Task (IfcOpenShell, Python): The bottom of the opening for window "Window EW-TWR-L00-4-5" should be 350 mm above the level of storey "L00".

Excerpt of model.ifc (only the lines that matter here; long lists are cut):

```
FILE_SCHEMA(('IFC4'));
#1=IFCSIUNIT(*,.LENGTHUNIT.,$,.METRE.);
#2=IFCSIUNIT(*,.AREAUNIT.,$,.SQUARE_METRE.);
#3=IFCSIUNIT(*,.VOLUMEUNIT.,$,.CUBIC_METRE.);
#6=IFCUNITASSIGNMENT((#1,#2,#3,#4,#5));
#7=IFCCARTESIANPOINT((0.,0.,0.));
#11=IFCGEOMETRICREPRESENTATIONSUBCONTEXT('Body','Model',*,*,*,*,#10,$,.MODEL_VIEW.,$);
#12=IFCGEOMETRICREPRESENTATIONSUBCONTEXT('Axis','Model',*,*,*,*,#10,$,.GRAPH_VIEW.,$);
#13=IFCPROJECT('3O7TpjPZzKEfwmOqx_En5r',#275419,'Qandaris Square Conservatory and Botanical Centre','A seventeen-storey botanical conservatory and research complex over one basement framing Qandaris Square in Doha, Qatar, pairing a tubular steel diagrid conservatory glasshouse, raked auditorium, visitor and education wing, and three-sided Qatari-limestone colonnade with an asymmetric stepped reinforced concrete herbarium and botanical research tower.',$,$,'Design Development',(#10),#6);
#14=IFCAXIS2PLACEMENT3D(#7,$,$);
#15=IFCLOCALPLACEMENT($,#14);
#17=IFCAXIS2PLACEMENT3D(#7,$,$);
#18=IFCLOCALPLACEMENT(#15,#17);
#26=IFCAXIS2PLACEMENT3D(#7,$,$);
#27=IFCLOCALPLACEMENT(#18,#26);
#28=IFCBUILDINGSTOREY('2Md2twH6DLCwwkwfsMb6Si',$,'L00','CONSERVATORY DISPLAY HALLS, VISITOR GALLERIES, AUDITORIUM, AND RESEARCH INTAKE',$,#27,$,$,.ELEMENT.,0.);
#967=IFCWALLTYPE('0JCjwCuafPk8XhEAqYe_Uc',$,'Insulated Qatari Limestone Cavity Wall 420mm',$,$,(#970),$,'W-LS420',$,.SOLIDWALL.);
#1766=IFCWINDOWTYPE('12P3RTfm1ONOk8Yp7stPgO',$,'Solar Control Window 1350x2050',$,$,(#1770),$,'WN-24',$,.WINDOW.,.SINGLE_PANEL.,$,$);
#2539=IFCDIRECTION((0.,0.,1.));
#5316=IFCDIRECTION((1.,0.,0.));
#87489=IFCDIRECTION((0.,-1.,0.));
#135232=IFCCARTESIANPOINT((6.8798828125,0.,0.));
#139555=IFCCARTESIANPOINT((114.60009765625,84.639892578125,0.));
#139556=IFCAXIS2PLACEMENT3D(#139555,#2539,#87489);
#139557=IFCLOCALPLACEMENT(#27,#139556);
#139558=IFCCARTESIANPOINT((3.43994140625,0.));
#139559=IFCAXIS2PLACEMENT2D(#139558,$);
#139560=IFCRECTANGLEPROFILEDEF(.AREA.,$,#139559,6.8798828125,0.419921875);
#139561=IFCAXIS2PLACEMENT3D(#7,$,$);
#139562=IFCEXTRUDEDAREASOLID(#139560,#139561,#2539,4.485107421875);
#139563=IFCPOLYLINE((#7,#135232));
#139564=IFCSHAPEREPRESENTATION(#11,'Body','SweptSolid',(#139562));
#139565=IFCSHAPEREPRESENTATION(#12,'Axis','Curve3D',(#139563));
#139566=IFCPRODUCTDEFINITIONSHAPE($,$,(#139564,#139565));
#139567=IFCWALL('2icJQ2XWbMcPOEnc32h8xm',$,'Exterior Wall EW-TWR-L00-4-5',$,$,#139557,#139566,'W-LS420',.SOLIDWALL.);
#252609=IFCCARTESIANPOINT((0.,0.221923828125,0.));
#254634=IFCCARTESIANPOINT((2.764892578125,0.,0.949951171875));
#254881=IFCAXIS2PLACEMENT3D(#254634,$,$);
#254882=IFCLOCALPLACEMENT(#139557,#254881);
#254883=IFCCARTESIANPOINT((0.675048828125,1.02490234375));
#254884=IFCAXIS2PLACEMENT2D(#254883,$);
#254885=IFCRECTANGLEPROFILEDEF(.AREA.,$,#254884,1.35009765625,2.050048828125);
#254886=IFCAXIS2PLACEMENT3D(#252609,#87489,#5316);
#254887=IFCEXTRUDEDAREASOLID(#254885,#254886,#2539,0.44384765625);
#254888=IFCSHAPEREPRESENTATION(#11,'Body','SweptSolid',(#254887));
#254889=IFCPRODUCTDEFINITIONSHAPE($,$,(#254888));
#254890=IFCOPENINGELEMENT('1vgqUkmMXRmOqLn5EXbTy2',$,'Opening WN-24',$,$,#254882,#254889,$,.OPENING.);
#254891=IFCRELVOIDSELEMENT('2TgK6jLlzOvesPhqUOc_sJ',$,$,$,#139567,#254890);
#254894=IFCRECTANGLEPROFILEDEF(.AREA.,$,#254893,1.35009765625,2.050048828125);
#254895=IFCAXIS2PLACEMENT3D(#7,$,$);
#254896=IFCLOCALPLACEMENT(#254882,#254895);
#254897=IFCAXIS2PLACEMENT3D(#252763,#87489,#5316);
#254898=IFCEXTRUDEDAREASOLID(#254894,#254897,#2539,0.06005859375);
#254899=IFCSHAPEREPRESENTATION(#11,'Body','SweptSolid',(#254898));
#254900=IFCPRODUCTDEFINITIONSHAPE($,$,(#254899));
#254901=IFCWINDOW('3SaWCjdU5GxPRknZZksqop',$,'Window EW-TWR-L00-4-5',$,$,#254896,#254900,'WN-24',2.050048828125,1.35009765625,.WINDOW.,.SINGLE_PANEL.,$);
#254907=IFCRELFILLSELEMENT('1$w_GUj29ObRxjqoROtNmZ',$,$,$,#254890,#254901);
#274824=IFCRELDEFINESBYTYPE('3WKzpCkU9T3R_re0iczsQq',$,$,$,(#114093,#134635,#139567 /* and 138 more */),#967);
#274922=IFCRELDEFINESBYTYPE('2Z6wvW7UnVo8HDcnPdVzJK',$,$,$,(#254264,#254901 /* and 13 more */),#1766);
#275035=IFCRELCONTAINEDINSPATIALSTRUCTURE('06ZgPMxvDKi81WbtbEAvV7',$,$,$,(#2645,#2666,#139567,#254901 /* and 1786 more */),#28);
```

```python
import numpy as np
import ifcopenshell
import ifcopenshell.api.geometry
import ifcopenshell.geom
import ifcopenshell.util.element
import ifcopenshell.util.placement
import ifcopenshell.util.shape
import ifcopenshell.util.unit

model = ifcopenshell.open("model.ifc")
unit_scale = ifcopenshell.util.unit.calculate_unit_scale(model)

window = model.by_id(254901)
opening = window.FillsVoids[0].RelatingOpeningElement
storey = ifcopenshell.util.element.get_container(window, ifc_class="IfcBuildingStorey")
level = ifcopenshell.util.placement.get_local_placement(storey.ObjectPlacement)[2, 3]

# The opening's origin need not be at the sill, so measure its lowest point.
shape = ifcopenshell.geom.create_shape(ifcopenshell.geom.settings(), opening)
bottom = ifcopenshell.util.shape.get_shape_bottom_elevation(shape, shape.geometry) / unit_scale
dz = level + 0.35 - bottom

shift = np.array([0.0, 0.0, dz])
# The window is placed relative to its opening, so it follows when the opening moves.
matrix = ifcopenshell.util.placement.get_local_placement(opening.ObjectPlacement)
matrix[:3, 3] += shift
ifcopenshell.api.geometry.edit_object_placement(
    model, product=opening, matrix=matrix, is_si=False, should_transform_children=True
)

print(f"moved by {dz * unit_scale:+.3f} m")

model.write("model-out.ifc")
```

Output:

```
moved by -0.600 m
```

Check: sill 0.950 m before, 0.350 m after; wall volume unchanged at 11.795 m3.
